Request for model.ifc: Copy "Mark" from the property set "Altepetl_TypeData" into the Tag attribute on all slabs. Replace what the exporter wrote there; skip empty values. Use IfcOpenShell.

First a look at what the model holds.

```python
import ifcopenshell
import ifcopenshell.util.element

model = ifcopenshell.open("model.ifc")
print(model.schema)
slabs = model.by_type("IfcSlab")
print(len(slabs), "slabs")
for e in slabs[:8]:
    source = ifcopenshell.util.element.get_pset(e, "Altepetl_TypeData", "Mark")
    target = e.Tag
    print(e.id(), repr(source), repr(target), sep=" | ")
```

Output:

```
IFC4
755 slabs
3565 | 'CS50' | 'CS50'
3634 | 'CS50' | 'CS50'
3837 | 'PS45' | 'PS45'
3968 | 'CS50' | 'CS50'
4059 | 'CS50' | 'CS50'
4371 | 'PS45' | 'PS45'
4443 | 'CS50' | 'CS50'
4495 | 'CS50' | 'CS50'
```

```python
import ifcopenshell
import ifcopenshell.util.element

model = ifcopenshell.open("model.ifc")

count = 0
for e in model.by_type("IfcSlab"):
    value = ifcopenshell.util.element.get_pset(e, "Altepetl_TypeData", "Mark")
    current = e.Tag
    if not value or not value.strip() or current == value:
        continue
    e.Tag = value
    count += 1

print(count, "slabs updated")

model.write("model_edited.ifc")
```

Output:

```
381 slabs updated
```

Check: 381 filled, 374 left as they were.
